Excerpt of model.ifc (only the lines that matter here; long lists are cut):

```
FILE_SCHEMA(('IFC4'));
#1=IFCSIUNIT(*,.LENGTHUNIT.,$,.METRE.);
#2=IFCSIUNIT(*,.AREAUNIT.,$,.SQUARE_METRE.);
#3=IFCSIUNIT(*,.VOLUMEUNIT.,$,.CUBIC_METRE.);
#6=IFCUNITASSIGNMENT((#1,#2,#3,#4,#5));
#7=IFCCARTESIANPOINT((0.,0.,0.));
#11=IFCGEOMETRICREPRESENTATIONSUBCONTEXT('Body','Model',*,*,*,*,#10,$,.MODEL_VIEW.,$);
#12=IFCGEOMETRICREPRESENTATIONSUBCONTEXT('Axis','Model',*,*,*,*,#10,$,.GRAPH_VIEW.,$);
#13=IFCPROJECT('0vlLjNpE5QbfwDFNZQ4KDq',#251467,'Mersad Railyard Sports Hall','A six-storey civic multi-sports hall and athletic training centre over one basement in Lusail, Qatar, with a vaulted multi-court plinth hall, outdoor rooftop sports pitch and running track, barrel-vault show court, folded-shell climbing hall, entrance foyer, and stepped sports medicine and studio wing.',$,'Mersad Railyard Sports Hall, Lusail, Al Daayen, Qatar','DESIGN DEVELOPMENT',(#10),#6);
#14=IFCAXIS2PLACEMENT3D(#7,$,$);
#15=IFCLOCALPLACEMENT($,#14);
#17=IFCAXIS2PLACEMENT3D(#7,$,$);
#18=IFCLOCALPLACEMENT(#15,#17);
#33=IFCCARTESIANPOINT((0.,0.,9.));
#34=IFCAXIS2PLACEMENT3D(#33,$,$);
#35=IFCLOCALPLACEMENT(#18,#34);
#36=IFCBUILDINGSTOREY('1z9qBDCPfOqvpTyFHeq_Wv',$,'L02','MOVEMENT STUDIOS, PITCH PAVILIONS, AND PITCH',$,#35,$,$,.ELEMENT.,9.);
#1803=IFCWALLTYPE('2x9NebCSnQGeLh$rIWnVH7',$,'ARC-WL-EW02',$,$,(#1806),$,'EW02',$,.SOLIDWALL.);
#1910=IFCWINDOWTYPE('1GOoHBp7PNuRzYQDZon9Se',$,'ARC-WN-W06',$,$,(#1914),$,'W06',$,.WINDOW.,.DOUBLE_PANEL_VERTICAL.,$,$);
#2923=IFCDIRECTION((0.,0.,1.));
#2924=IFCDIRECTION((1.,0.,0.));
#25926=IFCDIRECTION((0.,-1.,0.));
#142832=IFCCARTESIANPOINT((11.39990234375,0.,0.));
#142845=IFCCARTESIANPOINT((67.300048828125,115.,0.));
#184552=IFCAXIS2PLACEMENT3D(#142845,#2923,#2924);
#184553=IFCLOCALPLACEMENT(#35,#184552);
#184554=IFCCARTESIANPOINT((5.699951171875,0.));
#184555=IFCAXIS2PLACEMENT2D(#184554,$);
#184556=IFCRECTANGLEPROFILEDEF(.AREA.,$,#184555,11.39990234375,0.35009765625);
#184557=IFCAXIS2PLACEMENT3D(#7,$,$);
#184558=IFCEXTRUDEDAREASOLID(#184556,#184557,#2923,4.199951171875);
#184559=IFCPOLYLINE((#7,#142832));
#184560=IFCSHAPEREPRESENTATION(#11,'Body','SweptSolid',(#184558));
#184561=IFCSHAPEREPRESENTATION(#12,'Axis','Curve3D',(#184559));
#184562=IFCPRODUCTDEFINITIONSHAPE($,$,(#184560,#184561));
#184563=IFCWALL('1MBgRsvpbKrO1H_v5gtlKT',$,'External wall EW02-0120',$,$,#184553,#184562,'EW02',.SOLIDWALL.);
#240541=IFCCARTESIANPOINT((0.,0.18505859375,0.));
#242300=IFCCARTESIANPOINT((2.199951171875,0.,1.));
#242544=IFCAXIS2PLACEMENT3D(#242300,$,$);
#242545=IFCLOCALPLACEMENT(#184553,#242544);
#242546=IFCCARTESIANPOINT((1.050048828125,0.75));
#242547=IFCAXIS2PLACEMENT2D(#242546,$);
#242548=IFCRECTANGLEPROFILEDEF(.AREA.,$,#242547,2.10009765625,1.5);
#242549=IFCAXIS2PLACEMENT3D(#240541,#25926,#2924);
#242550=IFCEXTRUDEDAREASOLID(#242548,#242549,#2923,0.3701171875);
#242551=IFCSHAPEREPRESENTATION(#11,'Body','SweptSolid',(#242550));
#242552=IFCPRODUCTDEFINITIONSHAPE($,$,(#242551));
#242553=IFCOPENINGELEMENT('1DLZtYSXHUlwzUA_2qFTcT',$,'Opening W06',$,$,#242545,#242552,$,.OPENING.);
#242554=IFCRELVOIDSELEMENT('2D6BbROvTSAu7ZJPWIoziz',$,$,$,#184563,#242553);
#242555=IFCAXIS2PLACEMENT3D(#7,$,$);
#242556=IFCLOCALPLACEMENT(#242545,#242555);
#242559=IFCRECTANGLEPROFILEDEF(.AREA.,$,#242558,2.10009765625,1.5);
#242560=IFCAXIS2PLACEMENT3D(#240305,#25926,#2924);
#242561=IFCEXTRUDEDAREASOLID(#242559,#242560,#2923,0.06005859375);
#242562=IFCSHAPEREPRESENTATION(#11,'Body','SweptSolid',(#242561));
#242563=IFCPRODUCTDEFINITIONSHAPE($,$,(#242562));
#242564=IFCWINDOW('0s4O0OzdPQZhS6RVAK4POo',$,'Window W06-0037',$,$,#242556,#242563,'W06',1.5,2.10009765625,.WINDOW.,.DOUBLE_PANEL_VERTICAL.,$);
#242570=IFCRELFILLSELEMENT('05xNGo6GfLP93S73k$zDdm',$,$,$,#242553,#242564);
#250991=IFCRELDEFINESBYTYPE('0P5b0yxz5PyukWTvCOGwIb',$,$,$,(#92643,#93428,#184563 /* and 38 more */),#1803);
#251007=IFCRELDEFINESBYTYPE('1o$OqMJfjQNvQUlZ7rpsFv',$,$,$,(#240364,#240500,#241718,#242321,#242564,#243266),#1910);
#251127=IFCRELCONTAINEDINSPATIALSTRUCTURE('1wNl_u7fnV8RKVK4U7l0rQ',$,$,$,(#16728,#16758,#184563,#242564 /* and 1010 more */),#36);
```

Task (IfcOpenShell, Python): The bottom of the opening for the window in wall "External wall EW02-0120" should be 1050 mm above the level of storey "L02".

```python
import numpy as np
import ifcopenshell
import ifcopenshell.api.geometry
import ifcopenshell.geom
import ifcopenshell.util.element
import ifcopenshell.util.placement
import ifcopenshell.util.shape
import ifcopenshell.util.unit

model = ifcopenshell.open("model.ifc")
unit_scale = ifcopenshell.util.unit.calculate_unit_scale(model)

window = model.by_guid("0s4O0OzdPQZhS6RVAK4POo")
opening = window.FillsVoids[0].RelatingOpeningElement
storey = ifcopenshell.util.element.get_container(window, ifc_class="IfcBuildingStorey")
level = ifcopenshell.util.placement.get_local_placement(storey.ObjectPlacement)[2, 3]

# The opening's origin need not be at the sill, so measure its lowest point.
shape = ifcopenshell.geom.create_shape(ifcopenshell.geom.settings(), opening)
bottom = ifcopenshell.util.shape.get_shape_bottom_elevation(shape, shape.geometry) / unit_scale
dz = level + 1.05 / unit_scale - bottom

shift = np.array([0.0, 0.0, dz])
# The window is placed relative to its opening, so it follows when the opening moves.
matrix = ifcopenshell.util.placement.get_local_placement(opening.ObjectPlacement)
matrix[:3, 3] += shift
ifcopenshell.api.geometry.edit_object_placement(
    model, product=opening, matrix=matrix, is_si=False, should_transform_children=True
)

print(f"moved by {dz * unit_scale:+.3f} m")

model.write("model_rev.ifc")
```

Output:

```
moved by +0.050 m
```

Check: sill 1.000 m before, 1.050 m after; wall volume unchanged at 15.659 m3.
